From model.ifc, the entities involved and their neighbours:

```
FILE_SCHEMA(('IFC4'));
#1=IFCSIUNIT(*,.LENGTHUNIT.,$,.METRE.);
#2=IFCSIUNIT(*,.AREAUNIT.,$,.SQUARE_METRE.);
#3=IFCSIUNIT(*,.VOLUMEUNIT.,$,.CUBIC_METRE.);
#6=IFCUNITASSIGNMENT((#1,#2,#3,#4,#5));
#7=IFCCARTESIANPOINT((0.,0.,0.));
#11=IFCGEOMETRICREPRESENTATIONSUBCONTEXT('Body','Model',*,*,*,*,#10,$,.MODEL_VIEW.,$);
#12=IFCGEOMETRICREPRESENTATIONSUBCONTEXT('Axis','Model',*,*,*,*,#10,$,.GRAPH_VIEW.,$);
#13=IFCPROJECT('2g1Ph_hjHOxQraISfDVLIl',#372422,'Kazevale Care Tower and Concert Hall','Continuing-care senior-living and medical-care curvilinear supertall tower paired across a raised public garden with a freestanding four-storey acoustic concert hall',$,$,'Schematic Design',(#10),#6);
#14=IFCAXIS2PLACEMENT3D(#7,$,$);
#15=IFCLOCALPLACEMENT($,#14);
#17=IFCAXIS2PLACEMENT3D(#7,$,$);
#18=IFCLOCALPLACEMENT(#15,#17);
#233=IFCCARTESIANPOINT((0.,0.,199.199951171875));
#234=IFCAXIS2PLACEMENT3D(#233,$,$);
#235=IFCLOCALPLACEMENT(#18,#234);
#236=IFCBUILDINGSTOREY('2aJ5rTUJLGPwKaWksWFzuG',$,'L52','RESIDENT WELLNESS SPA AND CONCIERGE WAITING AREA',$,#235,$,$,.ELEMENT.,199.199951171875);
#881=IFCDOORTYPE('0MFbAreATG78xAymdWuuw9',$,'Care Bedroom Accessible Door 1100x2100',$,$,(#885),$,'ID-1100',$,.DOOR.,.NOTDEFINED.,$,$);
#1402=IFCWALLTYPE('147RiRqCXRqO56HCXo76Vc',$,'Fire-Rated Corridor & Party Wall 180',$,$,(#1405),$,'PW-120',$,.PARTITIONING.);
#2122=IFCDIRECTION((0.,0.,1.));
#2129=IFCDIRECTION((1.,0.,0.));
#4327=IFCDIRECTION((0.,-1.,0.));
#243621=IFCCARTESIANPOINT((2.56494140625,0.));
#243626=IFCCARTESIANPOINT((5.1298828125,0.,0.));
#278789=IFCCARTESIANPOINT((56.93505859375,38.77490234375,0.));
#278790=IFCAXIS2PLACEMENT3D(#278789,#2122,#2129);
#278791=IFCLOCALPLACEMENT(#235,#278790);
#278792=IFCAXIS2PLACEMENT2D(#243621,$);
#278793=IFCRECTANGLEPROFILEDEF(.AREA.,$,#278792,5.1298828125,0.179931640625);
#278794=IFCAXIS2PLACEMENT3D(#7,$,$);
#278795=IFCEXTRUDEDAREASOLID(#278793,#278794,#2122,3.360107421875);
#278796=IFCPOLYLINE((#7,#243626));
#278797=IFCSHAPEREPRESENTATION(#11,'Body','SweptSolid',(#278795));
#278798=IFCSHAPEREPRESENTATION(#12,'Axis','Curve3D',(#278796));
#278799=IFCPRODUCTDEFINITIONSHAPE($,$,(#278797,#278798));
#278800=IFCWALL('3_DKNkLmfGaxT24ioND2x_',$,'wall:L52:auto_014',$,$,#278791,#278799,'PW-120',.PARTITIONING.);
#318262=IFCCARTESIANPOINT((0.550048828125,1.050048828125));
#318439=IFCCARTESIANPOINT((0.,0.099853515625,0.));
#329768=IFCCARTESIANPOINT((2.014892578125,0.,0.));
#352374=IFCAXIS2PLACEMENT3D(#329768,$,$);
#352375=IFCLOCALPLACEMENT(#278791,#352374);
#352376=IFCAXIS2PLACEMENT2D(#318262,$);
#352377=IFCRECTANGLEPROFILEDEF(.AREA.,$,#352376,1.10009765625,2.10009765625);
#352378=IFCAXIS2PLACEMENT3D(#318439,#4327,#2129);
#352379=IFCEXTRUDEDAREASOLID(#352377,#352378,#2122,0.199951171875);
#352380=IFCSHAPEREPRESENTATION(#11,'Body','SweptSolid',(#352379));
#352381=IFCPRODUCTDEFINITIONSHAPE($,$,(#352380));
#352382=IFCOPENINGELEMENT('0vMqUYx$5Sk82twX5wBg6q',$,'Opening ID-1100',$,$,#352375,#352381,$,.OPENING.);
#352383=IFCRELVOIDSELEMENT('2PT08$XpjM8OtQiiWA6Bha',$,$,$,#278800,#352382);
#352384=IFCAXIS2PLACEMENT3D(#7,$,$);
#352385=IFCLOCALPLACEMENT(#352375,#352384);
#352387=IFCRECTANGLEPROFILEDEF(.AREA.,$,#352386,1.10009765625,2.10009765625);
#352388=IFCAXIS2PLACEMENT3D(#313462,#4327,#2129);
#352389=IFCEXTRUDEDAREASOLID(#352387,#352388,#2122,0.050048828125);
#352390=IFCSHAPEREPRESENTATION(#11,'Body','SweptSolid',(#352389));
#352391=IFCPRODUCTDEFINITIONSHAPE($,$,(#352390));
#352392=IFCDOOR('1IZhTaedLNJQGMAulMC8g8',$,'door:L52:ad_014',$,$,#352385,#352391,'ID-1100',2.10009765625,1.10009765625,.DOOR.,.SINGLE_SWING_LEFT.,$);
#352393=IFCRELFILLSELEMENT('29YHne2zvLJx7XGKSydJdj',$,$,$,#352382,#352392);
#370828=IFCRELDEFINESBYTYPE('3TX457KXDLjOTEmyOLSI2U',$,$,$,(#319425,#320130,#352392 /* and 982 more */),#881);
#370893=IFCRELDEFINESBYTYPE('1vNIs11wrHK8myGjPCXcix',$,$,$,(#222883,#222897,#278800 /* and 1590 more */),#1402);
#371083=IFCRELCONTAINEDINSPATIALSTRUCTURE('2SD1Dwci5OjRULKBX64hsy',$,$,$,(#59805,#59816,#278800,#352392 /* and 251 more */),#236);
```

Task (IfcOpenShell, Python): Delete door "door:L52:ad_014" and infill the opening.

```python
import ifcopenshell
import ifcopenshell.api.feature
import ifcopenshell.api.root
import ifcopenshell.geom
import ifcopenshell.util.shape

model = ifcopenshell.open("model.ifc")
settings = ifcopenshell.geom.settings()


def volume(element):
    """Net volume in cubic metres, openings subtracted."""
    shape = ifcopenshell.geom.create_shape(settings, element)
    return ifcopenshell.util.shape.get_volume(shape.geometry)


door = model.by_id(352392)
opening = door.FillsVoids[0].RelatingOpeningElement
wall = opening.VoidsElements[0].RelatingBuildingElement
before = volume(wall)

ifcopenshell.api.root.remove_product(model, product=door)
ifcopenshell.api.feature.remove_feature(model, feature=opening)

after = volume(wall)

print(f"wall volume {before:.3f} -> {after:.3f} m3")

model.write("model_v2.ifc")
```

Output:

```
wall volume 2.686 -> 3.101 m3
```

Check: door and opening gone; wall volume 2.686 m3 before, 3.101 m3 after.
